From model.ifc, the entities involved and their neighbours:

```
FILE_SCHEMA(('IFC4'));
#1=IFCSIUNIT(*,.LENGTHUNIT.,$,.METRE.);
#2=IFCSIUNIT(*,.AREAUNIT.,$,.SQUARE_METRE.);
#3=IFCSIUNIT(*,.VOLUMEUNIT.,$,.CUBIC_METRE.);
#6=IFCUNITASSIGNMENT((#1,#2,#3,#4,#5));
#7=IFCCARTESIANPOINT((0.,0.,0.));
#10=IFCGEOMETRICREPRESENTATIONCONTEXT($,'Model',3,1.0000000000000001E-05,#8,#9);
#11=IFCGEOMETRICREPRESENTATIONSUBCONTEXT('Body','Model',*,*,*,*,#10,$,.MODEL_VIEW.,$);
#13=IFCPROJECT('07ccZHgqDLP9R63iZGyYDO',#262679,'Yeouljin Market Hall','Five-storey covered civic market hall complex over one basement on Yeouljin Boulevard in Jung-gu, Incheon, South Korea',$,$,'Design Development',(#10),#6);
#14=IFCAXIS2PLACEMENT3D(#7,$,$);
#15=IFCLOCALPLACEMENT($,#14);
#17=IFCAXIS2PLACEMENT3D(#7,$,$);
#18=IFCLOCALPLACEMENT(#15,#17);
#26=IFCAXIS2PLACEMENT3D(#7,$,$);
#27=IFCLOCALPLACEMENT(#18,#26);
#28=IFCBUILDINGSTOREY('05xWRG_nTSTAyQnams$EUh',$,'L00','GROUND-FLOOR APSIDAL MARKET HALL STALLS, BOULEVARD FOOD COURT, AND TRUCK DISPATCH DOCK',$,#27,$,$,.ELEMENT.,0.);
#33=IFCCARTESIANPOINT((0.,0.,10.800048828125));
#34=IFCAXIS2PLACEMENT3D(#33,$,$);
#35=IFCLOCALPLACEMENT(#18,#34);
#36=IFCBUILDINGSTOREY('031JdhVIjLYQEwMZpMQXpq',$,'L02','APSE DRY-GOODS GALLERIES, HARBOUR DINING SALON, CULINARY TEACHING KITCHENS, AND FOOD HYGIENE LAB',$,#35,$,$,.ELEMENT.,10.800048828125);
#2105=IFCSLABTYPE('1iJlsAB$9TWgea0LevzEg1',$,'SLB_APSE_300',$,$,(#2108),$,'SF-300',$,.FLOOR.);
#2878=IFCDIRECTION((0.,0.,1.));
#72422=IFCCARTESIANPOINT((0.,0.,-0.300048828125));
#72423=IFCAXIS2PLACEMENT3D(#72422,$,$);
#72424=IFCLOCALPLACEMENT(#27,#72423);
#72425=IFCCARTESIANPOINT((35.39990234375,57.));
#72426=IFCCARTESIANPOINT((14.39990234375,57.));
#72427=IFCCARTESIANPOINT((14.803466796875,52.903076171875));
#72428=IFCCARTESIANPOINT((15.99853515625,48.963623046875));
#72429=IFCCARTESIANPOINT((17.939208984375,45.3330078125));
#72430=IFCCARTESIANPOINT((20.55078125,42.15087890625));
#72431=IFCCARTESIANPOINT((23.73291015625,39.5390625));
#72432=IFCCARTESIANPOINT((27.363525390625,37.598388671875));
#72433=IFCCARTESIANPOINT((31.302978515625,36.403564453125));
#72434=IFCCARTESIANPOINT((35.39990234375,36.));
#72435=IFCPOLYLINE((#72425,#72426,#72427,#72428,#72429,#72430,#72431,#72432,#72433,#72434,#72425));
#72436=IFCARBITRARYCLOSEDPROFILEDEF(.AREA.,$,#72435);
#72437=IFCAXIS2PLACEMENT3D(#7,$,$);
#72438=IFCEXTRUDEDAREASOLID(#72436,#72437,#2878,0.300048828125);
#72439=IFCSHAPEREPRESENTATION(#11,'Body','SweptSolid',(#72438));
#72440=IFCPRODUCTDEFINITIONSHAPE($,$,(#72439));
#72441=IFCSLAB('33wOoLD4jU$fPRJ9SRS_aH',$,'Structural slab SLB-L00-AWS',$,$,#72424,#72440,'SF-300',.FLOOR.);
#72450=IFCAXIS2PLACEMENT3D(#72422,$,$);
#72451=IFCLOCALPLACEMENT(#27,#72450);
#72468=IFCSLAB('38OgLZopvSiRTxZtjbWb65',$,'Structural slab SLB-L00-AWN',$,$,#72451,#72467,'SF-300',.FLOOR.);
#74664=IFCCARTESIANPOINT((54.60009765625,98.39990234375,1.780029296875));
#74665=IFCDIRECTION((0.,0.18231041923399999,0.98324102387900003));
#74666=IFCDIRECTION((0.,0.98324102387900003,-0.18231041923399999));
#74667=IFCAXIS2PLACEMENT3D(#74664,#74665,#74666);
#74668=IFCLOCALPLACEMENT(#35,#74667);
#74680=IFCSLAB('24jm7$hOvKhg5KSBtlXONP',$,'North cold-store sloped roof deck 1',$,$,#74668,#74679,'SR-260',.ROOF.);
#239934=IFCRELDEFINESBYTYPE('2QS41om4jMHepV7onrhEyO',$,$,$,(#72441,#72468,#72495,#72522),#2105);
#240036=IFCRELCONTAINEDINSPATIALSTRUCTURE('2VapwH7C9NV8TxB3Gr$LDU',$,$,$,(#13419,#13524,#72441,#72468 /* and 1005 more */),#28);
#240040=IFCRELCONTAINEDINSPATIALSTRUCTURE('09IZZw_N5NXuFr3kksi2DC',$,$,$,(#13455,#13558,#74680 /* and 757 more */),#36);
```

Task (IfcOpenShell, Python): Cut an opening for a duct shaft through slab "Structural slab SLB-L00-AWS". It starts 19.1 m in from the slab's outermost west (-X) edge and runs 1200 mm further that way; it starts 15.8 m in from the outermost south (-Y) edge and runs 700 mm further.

```python
import numpy as np
import ifcopenshell
import ifcopenshell.api.feature
import ifcopenshell.api.geometry
import ifcopenshell.api.root
import ifcopenshell.geom
import ifcopenshell.util.placement
import ifcopenshell.util.representation
import ifcopenshell.util.shape
import ifcopenshell.util.unit

model = ifcopenshell.open("model.ifc")
unit_scale = ifcopenshell.util.unit.calculate_unit_scale(model)
settings = ifcopenshell.geom.settings()


def volume(element):
    """Net volume in cubic metres, openings subtracted."""
    shape = ifcopenshell.geom.create_shape(settings, element)
    return ifcopenshell.util.shape.get_volume(shape.geometry)


slab = model.by_id(72441)
before = volume(slab)

# Extent in the slab's own axes, in metres. The edges named are its -X and -Y sides.
slab_shape = ifcopenshell.geom.create_shape(settings, slab)
vertices = ifcopenshell.util.shape.get_vertices(slab_shape.geometry)
x_min, y_min, bottom = vertices.min(axis=0)
top = vertices[:, 2].max()

opening = ifcopenshell.api.root.create_entity(model, ifc_class="IfcOpeningElement", name="Duct shaft opening", predefined_type="OPENING")
context = ifcopenshell.util.representation.get_context(model, "Model", "Body", "MODEL_VIEW")
width, depth = 1.2, 0.7
outline = [(0.0, 0.0), (width, 0.0), (width, depth), (0.0, depth), (0.0, 0.0)]
# Overshoot both faces by 50 mm so the cut is clean.
shape = ifcopenshell.api.geometry.add_slab_representation(
    model, context=context, depth=top - bottom + 0.1, polyline=outline
)
ifcopenshell.api.geometry.assign_representation(model, product=opening, representation=shape)

matrix = ifcopenshell.util.placement.get_local_placement(slab.ObjectPlacement)
matrix[:, 3] = matrix @ np.append(np.array([x_min + 19.1, y_min + 15.8, bottom - 0.05]) / unit_scale, 1.0)
ifcopenshell.api.geometry.edit_object_placement(model, product=opening, matrix=matrix, is_si=False)
ifcopenshell.api.feature.add_feature(model, feature=opening, element=slab)

after = volume(slab)

print(f"slab volume {before:.3f} -> {after:.3f} m3")

model.write("model_edited.ifc")
```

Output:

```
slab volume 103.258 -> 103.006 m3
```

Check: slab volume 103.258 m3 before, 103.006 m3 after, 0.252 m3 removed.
